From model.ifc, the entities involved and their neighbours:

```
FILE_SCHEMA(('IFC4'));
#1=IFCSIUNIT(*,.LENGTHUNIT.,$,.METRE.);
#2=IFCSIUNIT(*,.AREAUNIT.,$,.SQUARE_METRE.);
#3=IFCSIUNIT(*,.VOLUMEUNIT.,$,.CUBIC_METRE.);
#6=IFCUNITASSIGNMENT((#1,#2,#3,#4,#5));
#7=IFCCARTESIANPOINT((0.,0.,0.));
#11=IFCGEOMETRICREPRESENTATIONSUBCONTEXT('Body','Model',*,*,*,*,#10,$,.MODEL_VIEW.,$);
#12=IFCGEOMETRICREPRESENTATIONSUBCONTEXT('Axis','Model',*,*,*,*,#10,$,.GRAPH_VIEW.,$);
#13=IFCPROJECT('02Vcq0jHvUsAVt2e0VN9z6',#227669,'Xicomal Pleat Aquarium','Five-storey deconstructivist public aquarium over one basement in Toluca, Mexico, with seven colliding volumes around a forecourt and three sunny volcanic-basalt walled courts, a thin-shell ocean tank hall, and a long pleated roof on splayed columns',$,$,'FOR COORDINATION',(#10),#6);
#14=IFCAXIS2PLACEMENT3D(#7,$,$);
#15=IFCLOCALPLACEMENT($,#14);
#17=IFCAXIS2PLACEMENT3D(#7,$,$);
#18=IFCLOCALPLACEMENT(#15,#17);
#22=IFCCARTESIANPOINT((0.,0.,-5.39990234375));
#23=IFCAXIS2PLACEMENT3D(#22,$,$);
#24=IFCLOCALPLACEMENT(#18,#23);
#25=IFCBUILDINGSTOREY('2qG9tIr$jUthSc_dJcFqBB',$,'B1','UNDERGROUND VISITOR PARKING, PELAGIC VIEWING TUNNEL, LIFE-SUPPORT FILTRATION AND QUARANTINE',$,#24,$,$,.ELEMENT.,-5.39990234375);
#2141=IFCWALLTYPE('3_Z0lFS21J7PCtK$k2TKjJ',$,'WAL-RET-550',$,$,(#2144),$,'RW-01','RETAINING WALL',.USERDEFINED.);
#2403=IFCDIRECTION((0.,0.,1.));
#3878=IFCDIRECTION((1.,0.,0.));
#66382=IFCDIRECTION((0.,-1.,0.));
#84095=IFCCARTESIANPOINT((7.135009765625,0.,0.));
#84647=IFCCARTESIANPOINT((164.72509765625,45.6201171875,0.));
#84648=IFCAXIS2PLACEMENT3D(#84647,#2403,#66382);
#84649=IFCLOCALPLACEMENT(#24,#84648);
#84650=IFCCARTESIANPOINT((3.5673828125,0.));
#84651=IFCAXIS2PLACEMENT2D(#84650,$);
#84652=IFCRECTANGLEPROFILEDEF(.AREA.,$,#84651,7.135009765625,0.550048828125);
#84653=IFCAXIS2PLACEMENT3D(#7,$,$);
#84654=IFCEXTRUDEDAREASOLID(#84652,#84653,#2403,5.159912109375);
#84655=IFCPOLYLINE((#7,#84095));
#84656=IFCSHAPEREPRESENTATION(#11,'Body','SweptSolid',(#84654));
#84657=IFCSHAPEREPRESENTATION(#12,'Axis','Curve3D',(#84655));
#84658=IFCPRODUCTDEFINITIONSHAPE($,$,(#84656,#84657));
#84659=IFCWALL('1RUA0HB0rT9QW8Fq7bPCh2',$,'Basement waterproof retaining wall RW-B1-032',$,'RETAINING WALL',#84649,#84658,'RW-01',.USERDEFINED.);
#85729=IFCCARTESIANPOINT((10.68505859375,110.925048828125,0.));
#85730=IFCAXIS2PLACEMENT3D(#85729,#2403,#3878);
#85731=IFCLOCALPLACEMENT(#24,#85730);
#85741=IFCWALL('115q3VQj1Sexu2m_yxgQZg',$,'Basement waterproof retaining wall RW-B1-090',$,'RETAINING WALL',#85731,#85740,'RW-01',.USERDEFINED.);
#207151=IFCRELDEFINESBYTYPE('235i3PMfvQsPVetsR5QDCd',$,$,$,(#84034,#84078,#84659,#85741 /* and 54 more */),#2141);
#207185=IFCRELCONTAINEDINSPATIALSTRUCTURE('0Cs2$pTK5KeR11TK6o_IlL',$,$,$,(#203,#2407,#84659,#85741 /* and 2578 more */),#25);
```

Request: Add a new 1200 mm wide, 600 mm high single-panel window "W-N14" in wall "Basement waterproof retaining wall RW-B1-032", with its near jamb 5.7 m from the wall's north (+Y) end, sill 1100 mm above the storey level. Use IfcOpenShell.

```python
import numpy as np
import ifcopenshell
import ifcopenshell.api.feature
import ifcopenshell.api.geometry
import ifcopenshell.api.root
import ifcopenshell.api.spatial
import ifcopenshell.geom
import ifcopenshell.util.element
import ifcopenshell.util.placement
import ifcopenshell.util.representation
import ifcopenshell.util.shape
import ifcopenshell.util.unit

model = ifcopenshell.open("model.ifc")
unit_scale = ifcopenshell.util.unit.calculate_unit_scale(model)
settings = ifcopenshell.geom.settings()


def volume(element):
    """Net volume in cubic metres, openings subtracted."""
    shape = ifcopenshell.geom.create_shape(settings, element)
    return ifcopenshell.util.shape.get_volume(shape.geometry)


wall = model.by_guid("1RUA0HB0rT9QW8Fq7bPCh2")
storey = ifcopenshell.util.element.get_container(wall, ifc_class="IfcBuildingStorey")
context = ifcopenshell.util.representation.get_context(model, "Model", "Body", "MODEL_VIEW")
before = volume(wall)

width, height, from_end, sill = 1.2, 0.6, 5.7, 1.1  # metres

# The wall runs along its own X axis, and the end named is its -X end.
wall_shape = ifcopenshell.geom.create_shape(settings, wall)
x, y, z = ifcopenshell.util.shape.get_vertices(wall_shape.geometry).T
start = x.min() + from_end
face, thickness = float(y.min()), float(y.max() - y.min())
wall_matrix = ifcopenshell.util.placement.get_local_placement(wall.ObjectPlacement)
level = ifcopenshell.util.placement.get_local_placement(storey.ObjectPlacement)[2, 3]


def in_wall(x, y):
    """Placement at x, y metres in the wall's axes, at sill height."""
    matrix = wall_matrix.copy()
    matrix[:, 3] = wall_matrix @ np.array([x / unit_scale, y / unit_scale, 0.0, 1.0])
    matrix[2, 3] = level + sill / unit_scale
    return matrix


# Opening: a box that overshoots both wall faces by 50 mm.
opening = ifcopenshell.api.root.create_entity(model, ifc_class="IfcOpeningElement", predefined_type="OPENING")
box = ifcopenshell.api.geometry.add_wall_representation(
    model, context=context, length=width, height=height, thickness=thickness + 0.1
)
ifcopenshell.api.geometry.assign_representation(model, product=opening, representation=box)
ifcopenshell.api.geometry.edit_object_placement(model, product=opening, matrix=in_wall(start, face - 0.05), is_si=False)
ifcopenshell.api.feature.add_feature(model, feature=opening, element=wall)

window = ifcopenshell.api.root.create_entity(model, ifc_class="IfcWindow", name="W-N14", predefined_type="WINDOW")
window.OverallWidth, window.OverallHeight = width / unit_scale, height / unit_scale
window.PartitioningType = "SINGLE_PANEL"
body = ifcopenshell.api.geometry.add_window_representation(
    model,
    context=context,
    overall_width=window.OverallWidth,
    overall_height=window.OverallHeight,
    partition_type="SINGLE_PANEL",
)
ifcopenshell.api.geometry.assign_representation(model, product=window, representation=body)
ifcopenshell.api.spatial.assign_container(model, products=[window], relating_structure=storey)
ifcopenshell.api.feature.add_filling(model, opening=opening, element=window)

# Centre the window in the wall's thickness.
ifcopenshell.api.geometry.edit_object_placement(model, product=window, matrix=in_wall(start, face), is_si=False)
window_shape = ifcopenshell.geom.create_shape(settings, window)
depth = ifcopenshell.util.shape.get_vertices(window_shape.geometry)[:, 1]
offset = face + thickness / 2 - (depth.min() + depth.max()) / 2
ifcopenshell.api.geometry.edit_object_placement(model, product=window, matrix=in_wall(start, offset), is_si=False)

after = volume(wall)

print(f"wall volume {before:.3f} -> {after:.3f} m3")

model.write("model_updated.ifc")
```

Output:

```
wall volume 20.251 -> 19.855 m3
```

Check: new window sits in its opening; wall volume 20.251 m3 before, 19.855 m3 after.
